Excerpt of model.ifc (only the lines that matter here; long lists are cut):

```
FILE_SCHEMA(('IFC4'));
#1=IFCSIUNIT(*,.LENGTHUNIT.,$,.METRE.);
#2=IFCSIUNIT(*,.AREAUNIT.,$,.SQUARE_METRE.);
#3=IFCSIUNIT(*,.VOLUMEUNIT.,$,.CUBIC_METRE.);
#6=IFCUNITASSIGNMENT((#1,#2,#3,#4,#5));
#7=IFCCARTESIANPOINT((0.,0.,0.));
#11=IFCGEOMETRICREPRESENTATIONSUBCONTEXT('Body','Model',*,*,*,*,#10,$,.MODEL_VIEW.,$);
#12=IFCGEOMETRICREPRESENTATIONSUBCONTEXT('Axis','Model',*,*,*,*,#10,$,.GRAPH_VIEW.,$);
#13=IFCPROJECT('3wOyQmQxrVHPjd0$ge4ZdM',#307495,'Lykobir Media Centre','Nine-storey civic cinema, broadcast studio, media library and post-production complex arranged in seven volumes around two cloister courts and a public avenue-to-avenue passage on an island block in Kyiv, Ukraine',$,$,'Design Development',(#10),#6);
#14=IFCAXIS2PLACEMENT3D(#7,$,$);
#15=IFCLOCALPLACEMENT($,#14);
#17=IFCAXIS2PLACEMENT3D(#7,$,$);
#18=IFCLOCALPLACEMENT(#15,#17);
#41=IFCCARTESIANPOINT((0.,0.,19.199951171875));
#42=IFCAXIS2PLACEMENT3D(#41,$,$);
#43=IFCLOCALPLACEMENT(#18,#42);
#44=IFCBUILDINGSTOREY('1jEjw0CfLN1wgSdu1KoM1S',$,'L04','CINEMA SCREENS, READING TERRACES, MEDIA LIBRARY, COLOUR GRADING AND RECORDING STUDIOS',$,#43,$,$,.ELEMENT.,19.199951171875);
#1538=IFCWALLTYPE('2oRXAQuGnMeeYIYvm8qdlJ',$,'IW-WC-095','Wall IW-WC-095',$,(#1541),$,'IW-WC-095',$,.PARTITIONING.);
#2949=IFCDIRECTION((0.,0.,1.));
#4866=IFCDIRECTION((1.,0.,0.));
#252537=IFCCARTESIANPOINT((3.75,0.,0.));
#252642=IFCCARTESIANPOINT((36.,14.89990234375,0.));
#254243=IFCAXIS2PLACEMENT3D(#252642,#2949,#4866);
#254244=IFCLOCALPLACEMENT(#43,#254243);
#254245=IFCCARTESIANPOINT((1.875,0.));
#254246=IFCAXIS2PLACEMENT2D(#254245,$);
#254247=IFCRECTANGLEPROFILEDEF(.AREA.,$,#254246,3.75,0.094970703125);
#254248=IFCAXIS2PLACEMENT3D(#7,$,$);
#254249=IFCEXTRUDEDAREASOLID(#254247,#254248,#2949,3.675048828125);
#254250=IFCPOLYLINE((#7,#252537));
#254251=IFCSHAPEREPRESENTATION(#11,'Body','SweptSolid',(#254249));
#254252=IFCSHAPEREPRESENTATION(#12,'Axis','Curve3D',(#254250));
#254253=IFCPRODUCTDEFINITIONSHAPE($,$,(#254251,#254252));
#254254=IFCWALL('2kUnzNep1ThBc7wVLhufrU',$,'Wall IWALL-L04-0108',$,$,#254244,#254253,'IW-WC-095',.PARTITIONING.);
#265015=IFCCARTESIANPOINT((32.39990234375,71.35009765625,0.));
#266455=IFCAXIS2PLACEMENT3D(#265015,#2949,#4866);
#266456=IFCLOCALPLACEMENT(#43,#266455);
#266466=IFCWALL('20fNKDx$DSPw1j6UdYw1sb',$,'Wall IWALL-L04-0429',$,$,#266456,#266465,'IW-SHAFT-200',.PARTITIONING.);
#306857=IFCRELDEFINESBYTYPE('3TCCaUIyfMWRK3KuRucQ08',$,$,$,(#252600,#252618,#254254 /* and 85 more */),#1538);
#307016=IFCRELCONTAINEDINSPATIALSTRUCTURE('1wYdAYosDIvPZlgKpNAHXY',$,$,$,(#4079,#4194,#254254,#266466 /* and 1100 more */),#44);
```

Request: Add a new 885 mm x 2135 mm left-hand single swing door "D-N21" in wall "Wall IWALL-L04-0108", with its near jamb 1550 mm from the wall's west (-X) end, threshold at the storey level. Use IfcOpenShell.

```python
import numpy as np
import ifcopenshell
import ifcopenshell.api.feature
import ifcopenshell.api.geometry
import ifcopenshell.api.root
import ifcopenshell.api.spatial
import ifcopenshell.geom
import ifcopenshell.util.element
import ifcopenshell.util.placement
import ifcopenshell.util.representation
import ifcopenshell.util.shape
import ifcopenshell.util.unit

model = ifcopenshell.open("model.ifc")
unit_scale = ifcopenshell.util.unit.calculate_unit_scale(model)
settings = ifcopenshell.geom.settings()


def volume(element):
    """Net volume in cubic metres, openings subtracted."""
    shape = ifcopenshell.geom.create_shape(settings, element)
    return ifcopenshell.util.shape.get_volume(shape.geometry)


wall = model.by_id(254254)
storey = ifcopenshell.util.element.get_container(wall, ifc_class="IfcBuildingStorey")
context = ifcopenshell.util.representation.get_context(model, "Model", "Body", "MODEL_VIEW")
before = volume(wall)

width, height, from_end, sill = 0.885, 2.135, 1.55, 0.0  # metres

# The wall runs along its own X axis, and the end named is its -X end.
wall_shape = ifcopenshell.geom.create_shape(settings, wall)
x, y, z = ifcopenshell.util.shape.get_vertices(wall_shape.geometry).T
start = x.min() + from_end
face, thickness = float(y.min()), float(y.max() - y.min())
wall_matrix = ifcopenshell.util.placement.get_local_placement(wall.ObjectPlacement)
level = ifcopenshell.util.placement.get_local_placement(storey.ObjectPlacement)[2, 3]


def in_wall(x, y):
    """Placement at x, y metres in the wall's axes, at sill height."""
    matrix = wall_matrix.copy()
    matrix[:, 3] = wall_matrix @ np.array([x / unit_scale, y / unit_scale, 0.0, 1.0])
    matrix[2, 3] = level + sill / unit_scale
    return matrix


# Opening: a box that overshoots both wall faces by 50 mm.
opening = ifcopenshell.api.root.create_entity(model, ifc_class="IfcOpeningElement", predefined_type="OPENING")
box = ifcopenshell.api.geometry.add_wall_representation(
    model, context=context, length=width, height=height, thickness=thickness + 0.1
)
ifcopenshell.api.geometry.assign_representation(model, product=opening, representation=box)
ifcopenshell.api.geometry.edit_object_placement(model, product=opening, matrix=in_wall(start, face - 0.05), is_si=False)
ifcopenshell.api.feature.add_feature(model, feature=opening, element=wall)

door = ifcopenshell.api.root.create_entity(model, ifc_class="IfcDoor", name="D-N21", predefined_type="DOOR")
door.OverallWidth, door.OverallHeight = width / unit_scale, height / unit_scale
door.OperationType = "SINGLE_SWING_LEFT"
body = ifcopenshell.api.geometry.add_door_representation(
    model,
    context=context,
    overall_width=door.OverallWidth,
    overall_height=door.OverallHeight,
    operation_type="SINGLE_SWING_LEFT",
    lining_properties={"LiningDepth": thickness / unit_scale, "ThresholdDepth": thickness / unit_scale},
)
ifcopenshell.api.geometry.assign_representation(model, product=door, representation=body)
ifcopenshell.api.spatial.assign_container(model, products=[door], relating_structure=storey)
ifcopenshell.api.feature.add_filling(model, opening=opening, element=door)

# The lining spans the wall, so the door starts at the wall face.
ifcopenshell.api.geometry.edit_object_placement(model, product=door, matrix=in_wall(start, face), is_si=False)

after = volume(wall)

print(f"wall volume {before:.3f} -> {after:.3f} m3")

model.write("model_rev.ifc")
```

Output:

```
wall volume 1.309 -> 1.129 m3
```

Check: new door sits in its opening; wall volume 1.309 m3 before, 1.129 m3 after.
